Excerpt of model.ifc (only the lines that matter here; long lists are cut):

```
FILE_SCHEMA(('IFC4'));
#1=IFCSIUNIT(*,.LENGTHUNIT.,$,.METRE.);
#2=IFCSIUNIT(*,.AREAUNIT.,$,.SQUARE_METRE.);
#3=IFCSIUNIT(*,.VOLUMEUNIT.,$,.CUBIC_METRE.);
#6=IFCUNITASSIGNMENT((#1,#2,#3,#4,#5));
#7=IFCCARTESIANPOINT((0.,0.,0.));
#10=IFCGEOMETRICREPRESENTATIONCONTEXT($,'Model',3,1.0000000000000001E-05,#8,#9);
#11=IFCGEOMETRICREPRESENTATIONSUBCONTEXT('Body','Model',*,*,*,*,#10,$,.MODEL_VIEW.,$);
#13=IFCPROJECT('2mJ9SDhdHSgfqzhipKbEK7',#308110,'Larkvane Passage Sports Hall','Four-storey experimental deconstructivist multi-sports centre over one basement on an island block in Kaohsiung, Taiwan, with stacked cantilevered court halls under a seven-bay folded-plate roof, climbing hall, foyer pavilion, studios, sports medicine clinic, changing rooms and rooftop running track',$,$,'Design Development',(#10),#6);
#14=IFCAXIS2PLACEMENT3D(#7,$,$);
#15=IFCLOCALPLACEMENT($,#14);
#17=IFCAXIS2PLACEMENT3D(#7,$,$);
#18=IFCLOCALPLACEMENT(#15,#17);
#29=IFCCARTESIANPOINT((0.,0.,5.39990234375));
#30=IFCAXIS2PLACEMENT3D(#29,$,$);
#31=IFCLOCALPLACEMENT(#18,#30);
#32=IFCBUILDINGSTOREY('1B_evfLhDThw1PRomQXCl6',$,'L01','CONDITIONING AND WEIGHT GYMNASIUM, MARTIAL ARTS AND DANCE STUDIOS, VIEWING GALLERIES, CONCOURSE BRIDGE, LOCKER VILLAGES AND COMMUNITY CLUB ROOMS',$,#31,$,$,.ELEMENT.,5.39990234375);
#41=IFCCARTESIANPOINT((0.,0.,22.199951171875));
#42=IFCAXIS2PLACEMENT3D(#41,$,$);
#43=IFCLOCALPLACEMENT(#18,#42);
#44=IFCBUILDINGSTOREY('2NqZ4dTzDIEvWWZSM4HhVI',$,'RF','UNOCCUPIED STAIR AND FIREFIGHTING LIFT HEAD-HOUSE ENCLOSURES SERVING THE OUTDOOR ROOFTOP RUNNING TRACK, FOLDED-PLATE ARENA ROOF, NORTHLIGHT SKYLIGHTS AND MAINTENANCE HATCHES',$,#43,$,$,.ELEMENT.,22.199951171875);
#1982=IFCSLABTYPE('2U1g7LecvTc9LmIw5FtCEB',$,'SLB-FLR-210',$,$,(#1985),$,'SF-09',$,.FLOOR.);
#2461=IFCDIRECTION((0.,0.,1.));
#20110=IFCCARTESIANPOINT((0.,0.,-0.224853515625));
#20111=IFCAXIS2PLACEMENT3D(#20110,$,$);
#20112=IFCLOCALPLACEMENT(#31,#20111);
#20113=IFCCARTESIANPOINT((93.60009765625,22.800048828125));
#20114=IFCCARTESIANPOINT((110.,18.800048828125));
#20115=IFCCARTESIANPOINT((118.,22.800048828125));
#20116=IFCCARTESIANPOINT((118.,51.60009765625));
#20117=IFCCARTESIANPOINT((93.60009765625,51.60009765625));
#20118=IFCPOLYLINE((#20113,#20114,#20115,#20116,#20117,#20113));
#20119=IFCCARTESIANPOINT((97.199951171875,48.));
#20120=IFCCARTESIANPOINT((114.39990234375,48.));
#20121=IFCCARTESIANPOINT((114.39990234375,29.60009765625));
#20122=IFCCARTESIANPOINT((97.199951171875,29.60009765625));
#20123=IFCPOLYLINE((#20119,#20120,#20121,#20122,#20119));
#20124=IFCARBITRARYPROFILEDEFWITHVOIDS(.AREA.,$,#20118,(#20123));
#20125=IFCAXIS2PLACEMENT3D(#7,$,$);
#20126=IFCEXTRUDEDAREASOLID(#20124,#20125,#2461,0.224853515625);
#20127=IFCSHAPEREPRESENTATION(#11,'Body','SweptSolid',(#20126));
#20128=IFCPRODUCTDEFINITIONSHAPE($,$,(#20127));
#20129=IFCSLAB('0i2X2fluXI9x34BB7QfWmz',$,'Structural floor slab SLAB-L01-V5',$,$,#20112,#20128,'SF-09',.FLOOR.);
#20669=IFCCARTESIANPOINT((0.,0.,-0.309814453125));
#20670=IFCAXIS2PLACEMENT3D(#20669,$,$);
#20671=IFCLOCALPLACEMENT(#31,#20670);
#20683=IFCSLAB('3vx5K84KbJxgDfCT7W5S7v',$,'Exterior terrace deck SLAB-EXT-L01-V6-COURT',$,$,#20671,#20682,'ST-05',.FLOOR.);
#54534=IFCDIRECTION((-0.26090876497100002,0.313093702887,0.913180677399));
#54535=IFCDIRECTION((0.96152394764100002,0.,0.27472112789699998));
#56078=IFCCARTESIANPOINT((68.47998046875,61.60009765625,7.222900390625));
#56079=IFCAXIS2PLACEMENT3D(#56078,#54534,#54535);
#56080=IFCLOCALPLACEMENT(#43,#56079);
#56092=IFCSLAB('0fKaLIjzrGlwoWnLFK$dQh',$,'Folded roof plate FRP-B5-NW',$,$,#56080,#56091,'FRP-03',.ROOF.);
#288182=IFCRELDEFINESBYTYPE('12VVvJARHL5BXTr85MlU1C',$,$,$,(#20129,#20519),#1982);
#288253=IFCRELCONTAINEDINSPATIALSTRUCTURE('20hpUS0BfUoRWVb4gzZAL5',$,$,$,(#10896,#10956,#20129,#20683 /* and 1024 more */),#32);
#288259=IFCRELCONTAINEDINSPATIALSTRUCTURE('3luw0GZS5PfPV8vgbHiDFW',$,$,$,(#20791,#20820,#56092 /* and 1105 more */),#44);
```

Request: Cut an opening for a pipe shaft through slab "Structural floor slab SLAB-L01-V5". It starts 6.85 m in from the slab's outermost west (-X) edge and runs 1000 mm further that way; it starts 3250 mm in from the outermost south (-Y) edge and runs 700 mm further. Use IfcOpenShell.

```python
import numpy as np
import ifcopenshell
import ifcopenshell.api.feature
import ifcopenshell.api.geometry
import ifcopenshell.api.root
import ifcopenshell.geom
import ifcopenshell.util.placement
import ifcopenshell.util.representation
import ifcopenshell.util.shape
import ifcopenshell.util.unit

model = ifcopenshell.open("model.ifc")
unit_scale = ifcopenshell.util.unit.calculate_unit_scale(model)
settings = ifcopenshell.geom.settings()


def volume(element):
    """Net volume in cubic metres, openings subtracted."""
    shape = ifcopenshell.geom.create_shape(settings, element)
    return ifcopenshell.util.shape.get_volume(shape.geometry)


slab = model.by_guid("0i2X2fluXI9x34BB7QfWmz")
before = volume(slab)

# Extent in the slab's own axes, in metres. The edges named are its -X and -Y sides.
slab_shape = ifcopenshell.geom.create_shape(settings, slab)
vertices = ifcopenshell.util.shape.get_vertices(slab_shape.geometry)
x_min, y_min, bottom = vertices.min(axis=0)
top = vertices[:, 2].max()

opening = ifcopenshell.api.root.create_entity(model, ifc_class="IfcOpeningElement", name="Pipe shaft opening", predefined_type="OPENING")
context = ifcopenshell.util.representation.get_context(model, "Model", "Body", "MODEL_VIEW")
width, depth = 1, 0.7
outline = [(0.0, 0.0), (width, 0.0), (width, depth), (0.0, depth), (0.0, 0.0)]
# Overshoot both faces by 50 mm so the cut is clean.
shape = ifcopenshell.api.geometry.add_slab_representation(
    model, context=context, depth=top - bottom + 0.1, polyline=outline
)
ifcopenshell.api.geometry.assign_representation(model, product=opening, representation=shape)

matrix = ifcopenshell.util.placement.get_local_placement(slab.ObjectPlacement)
matrix[:, 3] = matrix @ np.append(np.array([x_min + 6.85, y_min + 3.25, bottom - 0.05]) / unit_scale, 1.0)
ifcopenshell.api.geometry.edit_object_placement(model, product=opening, matrix=matrix, is_si=False)
ifcopenshell.api.feature.add_feature(model, feature=opening, element=slab)

after = volume(slab)

print(f"slab volume {before:.3f} -> {after:.3f} m3")

model.write("model_edited.ifc")
```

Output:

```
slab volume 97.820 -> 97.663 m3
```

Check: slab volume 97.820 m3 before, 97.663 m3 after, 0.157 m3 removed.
